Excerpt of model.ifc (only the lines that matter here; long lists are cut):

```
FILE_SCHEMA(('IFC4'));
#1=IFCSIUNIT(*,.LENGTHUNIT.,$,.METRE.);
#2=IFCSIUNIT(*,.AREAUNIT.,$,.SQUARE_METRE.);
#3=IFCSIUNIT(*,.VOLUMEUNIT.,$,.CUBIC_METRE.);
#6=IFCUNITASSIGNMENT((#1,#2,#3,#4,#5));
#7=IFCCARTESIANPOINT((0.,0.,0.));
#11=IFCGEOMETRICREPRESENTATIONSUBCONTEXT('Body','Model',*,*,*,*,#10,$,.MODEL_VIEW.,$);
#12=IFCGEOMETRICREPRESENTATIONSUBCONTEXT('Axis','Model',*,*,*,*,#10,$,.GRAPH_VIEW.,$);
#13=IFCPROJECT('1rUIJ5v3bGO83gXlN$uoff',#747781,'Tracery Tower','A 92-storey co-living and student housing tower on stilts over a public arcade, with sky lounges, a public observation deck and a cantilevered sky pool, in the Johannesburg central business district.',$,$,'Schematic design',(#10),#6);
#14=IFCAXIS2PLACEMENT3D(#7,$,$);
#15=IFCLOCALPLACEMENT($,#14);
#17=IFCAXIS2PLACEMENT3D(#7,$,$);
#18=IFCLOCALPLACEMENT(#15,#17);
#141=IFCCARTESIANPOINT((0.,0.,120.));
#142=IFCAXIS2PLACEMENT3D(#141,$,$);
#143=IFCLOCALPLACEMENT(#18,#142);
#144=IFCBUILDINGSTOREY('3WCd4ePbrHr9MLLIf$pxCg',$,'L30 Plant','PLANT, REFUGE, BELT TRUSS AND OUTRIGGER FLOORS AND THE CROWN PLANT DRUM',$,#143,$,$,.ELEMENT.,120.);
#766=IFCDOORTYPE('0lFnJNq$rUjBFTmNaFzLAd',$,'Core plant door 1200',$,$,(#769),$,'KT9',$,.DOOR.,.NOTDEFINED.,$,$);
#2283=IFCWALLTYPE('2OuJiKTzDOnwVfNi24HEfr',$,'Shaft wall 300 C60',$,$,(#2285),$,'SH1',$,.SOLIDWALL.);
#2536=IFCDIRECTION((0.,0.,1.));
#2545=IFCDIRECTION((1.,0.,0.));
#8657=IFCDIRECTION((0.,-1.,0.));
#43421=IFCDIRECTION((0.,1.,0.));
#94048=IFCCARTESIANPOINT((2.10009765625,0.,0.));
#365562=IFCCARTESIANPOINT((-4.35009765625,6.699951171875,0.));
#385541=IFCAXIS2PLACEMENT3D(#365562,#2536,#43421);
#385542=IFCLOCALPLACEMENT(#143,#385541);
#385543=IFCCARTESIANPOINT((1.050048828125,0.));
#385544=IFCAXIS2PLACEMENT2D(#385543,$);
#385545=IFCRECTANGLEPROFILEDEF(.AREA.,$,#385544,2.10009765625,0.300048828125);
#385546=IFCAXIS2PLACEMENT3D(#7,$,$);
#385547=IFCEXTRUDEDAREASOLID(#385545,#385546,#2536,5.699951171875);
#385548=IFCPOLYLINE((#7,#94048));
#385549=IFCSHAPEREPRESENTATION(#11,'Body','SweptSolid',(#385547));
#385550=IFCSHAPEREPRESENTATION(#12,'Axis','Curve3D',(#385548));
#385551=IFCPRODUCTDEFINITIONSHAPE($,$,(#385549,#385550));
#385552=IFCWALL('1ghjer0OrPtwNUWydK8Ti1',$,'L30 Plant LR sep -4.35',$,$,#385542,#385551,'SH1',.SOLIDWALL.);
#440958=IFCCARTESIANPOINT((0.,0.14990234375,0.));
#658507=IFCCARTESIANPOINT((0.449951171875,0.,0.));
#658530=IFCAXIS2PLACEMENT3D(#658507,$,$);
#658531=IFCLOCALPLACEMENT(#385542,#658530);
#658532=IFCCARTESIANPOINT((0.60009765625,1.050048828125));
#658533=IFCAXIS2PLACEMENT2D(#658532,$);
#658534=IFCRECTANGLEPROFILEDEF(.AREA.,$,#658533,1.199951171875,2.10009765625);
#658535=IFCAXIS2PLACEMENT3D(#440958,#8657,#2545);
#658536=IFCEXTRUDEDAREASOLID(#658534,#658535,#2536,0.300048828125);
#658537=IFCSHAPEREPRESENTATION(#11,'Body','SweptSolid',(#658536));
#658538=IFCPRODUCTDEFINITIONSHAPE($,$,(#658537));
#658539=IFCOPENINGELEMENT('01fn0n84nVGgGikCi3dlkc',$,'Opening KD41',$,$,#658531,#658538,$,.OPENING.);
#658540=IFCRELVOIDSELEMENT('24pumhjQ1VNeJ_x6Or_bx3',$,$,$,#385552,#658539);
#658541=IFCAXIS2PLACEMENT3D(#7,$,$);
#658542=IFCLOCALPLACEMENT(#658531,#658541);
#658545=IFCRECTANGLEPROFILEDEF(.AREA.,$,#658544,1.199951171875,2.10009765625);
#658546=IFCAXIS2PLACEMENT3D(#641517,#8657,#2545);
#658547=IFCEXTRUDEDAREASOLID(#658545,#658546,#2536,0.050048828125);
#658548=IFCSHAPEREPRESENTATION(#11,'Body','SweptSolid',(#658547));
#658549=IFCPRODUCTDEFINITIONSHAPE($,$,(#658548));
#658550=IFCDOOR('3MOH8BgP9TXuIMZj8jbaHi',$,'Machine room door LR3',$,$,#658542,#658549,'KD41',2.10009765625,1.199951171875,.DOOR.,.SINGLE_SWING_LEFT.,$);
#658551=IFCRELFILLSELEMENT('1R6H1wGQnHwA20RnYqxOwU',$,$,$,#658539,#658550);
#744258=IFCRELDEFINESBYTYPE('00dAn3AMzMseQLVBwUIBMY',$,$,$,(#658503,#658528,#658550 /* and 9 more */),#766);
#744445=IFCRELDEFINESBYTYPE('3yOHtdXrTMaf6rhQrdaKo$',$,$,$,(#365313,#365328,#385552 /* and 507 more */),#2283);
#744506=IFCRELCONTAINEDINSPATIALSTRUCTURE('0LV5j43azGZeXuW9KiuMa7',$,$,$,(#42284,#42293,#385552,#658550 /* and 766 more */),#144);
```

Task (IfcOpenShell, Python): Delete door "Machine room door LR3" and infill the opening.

```python
import ifcopenshell
import ifcopenshell.api.feature
import ifcopenshell.api.root
import ifcopenshell.geom
import ifcopenshell.util.shape

model = ifcopenshell.open("model.ifc")
settings = ifcopenshell.geom.settings()


def volume(element):
    """Net volume in cubic metres, openings subtracted."""
    shape = ifcopenshell.geom.create_shape(settings, element)
    return ifcopenshell.util.shape.get_volume(shape.geometry)


door = model.by_guid("3MOH8BgP9TXuIMZj8jbaHi")
opening = door.FillsVoids[0].RelatingOpeningElement
wall = opening.VoidsElements[0].RelatingBuildingElement
before = volume(wall)

ifcopenshell.api.root.remove_product(model, product=door)
ifcopenshell.api.feature.remove_feature(model, feature=opening)

after = volume(wall)

print(f"wall volume {before:.3f} -> {after:.3f} m3")

model.write("model_v2.ifc")
```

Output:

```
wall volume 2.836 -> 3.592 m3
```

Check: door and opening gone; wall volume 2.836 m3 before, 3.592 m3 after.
